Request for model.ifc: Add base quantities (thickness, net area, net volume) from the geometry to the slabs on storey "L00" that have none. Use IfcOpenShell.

First a look at what the model holds.

```python
import ifcopenshell
import ifcopenshell.util.element
import ifcopenshell.util.unit

model = ifcopenshell.open("model.ifc")
print(model.schema)
for unit_type in ("LENGTHUNIT", "AREAUNIT", "VOLUMEUNIT"):
    print(unit_type, ifcopenshell.util.unit.calculate_unit_scale(model, unit_type))
storey = next(s for s in model.by_type("IfcBuildingStorey") if s.Name == "L00")
slabs = [e for e in ifcopenshell.util.element.get_decomposition(storey) if e.is_a("IfcSlab")]
for e in sorted(slabs, key=lambda e: e.id()):
    print(e.id(), e.is_a(), e.Name, list(ifcopenshell.util.element.get_psets(e, qtos_only=True)), sep=" | ")
```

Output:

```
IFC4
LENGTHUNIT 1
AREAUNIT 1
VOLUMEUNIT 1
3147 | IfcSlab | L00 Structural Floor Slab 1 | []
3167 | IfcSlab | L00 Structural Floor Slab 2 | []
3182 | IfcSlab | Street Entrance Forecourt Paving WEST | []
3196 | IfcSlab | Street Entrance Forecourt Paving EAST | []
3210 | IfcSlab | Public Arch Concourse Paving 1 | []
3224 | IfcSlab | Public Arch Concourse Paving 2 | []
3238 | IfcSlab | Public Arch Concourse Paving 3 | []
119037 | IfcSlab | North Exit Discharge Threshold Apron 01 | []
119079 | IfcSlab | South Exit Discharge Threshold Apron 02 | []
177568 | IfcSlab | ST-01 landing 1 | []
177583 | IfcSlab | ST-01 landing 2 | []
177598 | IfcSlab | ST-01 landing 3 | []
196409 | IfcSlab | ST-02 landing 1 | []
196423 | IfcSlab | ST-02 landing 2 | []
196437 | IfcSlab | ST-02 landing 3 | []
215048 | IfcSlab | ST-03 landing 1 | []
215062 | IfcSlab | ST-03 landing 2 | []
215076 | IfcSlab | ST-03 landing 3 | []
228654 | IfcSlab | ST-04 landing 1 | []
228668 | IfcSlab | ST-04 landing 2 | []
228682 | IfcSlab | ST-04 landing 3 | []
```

```python
import ifcopenshell
import ifcopenshell.api.pset
import ifcopenshell.geom
import ifcopenshell.util.element
import ifcopenshell.util.shape
import ifcopenshell.util.unit

model = ifcopenshell.open("model.ifc")
unit_scale = ifcopenshell.util.unit.calculate_unit_scale(model)
area_scale = ifcopenshell.util.unit.calculate_unit_scale(model, "AREAUNIT")
volume_scale = ifcopenshell.util.unit.calculate_unit_scale(model, "VOLUMEUNIT")
settings = ifcopenshell.geom.settings()

storey = next(s for s in model.by_type("IfcBuildingStorey") if s.Name == "L00")
slabs = [e for e in ifcopenshell.util.element.get_decomposition(storey) if e.is_a("IfcSlab")]

for e in sorted(slabs, key=lambda e: e.id()):
    if ifcopenshell.util.element.get_psets(e, qtos_only=True, should_inherit=False):
        continue
    # Geometry comes back in metres, in the element's own axes.
    shape = ifcopenshell.geom.create_shape(settings, e)
    values = {
        "Width": ifcopenshell.util.shape.get_z(shape.geometry) / unit_scale,
        "NetArea": ifcopenshell.util.shape.get_footprint_area(shape.geometry) / area_scale,
        "NetVolume": ifcopenshell.util.shape.get_volume(shape.geometry) / volume_scale,
    }
    qto = ifcopenshell.api.pset.add_qto(model, product=e, name="Qto_SlabBaseQuantities")
    ifcopenshell.api.pset.edit_qto(model, qto=qto, properties=values)
    print(e.id(), {k: round(v, 3) for k, v in values.items()})

model.write("model_edited.ifc")
```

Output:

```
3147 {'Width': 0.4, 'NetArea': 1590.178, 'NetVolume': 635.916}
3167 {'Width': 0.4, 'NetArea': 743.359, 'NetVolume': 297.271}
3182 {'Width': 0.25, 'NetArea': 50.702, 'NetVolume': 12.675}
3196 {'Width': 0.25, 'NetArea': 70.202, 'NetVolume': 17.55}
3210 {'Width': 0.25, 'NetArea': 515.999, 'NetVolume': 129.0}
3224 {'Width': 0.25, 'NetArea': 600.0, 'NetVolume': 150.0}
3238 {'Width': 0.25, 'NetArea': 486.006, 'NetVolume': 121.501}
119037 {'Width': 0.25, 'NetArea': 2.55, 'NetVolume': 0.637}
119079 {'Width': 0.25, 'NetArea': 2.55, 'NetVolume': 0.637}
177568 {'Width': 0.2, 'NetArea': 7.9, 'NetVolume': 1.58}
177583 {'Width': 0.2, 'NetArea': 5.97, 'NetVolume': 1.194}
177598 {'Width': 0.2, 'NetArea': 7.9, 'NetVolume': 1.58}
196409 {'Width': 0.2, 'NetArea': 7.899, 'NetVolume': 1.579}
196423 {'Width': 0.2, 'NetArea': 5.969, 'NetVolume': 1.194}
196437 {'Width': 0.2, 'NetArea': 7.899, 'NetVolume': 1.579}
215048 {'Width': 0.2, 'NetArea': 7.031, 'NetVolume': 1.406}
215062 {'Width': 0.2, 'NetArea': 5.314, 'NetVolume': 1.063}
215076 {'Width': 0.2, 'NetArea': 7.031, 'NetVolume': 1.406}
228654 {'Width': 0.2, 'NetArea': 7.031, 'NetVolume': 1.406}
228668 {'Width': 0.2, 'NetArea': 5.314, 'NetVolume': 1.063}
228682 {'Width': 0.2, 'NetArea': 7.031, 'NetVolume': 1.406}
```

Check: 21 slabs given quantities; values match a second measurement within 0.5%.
